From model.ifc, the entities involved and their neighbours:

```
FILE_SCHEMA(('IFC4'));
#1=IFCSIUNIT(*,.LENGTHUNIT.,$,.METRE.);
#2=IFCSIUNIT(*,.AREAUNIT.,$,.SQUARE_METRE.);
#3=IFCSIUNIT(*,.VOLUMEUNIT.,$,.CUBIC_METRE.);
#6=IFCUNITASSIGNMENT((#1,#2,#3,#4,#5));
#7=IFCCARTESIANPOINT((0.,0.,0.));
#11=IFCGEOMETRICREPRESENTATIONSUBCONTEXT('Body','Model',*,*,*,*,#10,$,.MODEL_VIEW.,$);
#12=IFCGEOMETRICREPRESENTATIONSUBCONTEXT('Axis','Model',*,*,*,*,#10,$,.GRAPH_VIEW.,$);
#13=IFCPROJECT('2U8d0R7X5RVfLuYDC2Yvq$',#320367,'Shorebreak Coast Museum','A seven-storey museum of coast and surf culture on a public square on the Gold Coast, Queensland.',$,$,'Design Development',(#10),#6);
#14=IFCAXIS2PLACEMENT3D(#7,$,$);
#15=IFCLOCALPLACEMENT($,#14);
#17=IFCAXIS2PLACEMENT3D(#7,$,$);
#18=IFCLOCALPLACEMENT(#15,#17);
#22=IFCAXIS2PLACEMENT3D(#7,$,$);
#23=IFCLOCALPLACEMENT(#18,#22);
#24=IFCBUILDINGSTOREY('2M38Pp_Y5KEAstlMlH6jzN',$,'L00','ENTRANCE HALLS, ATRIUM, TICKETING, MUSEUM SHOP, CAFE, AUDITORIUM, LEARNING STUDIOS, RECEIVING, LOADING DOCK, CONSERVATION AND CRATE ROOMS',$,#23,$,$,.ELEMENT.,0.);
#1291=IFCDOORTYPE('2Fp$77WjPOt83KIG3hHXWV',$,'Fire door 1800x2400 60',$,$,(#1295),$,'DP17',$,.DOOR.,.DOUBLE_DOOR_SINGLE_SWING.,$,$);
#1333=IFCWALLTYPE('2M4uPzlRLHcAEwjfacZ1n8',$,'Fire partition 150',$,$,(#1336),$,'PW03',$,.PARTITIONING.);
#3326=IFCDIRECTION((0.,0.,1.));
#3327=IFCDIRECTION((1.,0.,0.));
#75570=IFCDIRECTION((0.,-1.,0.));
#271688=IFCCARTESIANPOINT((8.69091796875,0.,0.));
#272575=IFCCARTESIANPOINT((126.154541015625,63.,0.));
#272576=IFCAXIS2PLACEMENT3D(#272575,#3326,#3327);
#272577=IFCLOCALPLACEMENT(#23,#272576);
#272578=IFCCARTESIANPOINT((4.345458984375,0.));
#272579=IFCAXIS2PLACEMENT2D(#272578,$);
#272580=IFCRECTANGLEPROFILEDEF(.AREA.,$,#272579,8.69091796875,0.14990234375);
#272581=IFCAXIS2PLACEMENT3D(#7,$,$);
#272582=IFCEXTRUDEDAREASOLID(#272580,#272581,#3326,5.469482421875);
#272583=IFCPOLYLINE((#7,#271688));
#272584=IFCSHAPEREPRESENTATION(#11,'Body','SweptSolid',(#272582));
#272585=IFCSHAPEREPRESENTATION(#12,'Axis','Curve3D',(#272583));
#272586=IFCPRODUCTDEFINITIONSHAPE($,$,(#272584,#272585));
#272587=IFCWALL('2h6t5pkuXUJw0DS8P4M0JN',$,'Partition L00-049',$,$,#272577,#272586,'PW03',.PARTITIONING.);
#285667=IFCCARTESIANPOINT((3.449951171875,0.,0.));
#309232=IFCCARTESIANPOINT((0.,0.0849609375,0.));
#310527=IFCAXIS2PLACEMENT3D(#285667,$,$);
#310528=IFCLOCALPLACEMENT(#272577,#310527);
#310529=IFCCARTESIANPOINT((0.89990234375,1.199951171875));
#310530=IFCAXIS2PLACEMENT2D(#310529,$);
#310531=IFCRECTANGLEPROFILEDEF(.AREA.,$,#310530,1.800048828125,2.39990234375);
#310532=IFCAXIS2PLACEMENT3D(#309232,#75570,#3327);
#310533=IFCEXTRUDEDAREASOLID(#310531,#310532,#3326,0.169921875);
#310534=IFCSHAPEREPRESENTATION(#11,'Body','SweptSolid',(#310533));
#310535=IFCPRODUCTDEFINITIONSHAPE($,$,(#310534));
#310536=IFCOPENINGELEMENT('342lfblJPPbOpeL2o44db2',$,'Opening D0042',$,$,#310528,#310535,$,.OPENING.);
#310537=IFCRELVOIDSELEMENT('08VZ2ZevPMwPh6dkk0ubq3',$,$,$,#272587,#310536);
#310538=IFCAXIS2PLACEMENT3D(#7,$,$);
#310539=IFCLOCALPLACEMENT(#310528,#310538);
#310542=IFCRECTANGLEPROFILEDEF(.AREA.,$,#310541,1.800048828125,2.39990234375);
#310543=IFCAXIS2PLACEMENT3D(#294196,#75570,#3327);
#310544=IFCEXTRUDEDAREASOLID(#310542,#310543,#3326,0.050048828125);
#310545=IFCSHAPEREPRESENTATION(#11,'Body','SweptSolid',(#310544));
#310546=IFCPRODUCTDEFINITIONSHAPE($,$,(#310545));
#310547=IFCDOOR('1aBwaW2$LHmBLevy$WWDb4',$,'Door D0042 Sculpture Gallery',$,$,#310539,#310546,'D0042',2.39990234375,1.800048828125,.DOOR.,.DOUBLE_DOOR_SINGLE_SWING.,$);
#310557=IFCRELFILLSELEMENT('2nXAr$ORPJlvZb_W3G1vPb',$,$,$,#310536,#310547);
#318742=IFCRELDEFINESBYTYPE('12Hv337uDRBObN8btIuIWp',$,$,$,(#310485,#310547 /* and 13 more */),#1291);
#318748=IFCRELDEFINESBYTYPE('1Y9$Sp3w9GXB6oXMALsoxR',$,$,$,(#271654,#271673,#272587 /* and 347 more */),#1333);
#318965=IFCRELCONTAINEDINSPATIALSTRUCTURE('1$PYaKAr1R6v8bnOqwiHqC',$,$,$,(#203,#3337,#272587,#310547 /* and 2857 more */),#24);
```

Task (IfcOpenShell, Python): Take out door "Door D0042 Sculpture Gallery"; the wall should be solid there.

```python
import ifcopenshell
import ifcopenshell.api.feature
import ifcopenshell.api.root
import ifcopenshell.geom
import ifcopenshell.util.shape

model = ifcopenshell.open("model.ifc")
settings = ifcopenshell.geom.settings()


def volume(element):
    """Net volume in cubic metres, openings subtracted."""
    shape = ifcopenshell.geom.create_shape(settings, element)
    return ifcopenshell.util.shape.get_volume(shape.geometry)


door = model.by_guid("1aBwaW2$LHmBLevy$WWDb4")
opening = door.FillsVoids[0].RelatingOpeningElement
wall = opening.VoidsElements[0].RelatingBuildingElement
before = volume(wall)

ifcopenshell.api.root.remove_product(model, product=door)
ifcopenshell.api.feature.remove_feature(model, feature=opening)

after = volume(wall)

print(f"wall volume {before:.3f} -> {after:.3f} m3")

model.write("model-out.ifc")
```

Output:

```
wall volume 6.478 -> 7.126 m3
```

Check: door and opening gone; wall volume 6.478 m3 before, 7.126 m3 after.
